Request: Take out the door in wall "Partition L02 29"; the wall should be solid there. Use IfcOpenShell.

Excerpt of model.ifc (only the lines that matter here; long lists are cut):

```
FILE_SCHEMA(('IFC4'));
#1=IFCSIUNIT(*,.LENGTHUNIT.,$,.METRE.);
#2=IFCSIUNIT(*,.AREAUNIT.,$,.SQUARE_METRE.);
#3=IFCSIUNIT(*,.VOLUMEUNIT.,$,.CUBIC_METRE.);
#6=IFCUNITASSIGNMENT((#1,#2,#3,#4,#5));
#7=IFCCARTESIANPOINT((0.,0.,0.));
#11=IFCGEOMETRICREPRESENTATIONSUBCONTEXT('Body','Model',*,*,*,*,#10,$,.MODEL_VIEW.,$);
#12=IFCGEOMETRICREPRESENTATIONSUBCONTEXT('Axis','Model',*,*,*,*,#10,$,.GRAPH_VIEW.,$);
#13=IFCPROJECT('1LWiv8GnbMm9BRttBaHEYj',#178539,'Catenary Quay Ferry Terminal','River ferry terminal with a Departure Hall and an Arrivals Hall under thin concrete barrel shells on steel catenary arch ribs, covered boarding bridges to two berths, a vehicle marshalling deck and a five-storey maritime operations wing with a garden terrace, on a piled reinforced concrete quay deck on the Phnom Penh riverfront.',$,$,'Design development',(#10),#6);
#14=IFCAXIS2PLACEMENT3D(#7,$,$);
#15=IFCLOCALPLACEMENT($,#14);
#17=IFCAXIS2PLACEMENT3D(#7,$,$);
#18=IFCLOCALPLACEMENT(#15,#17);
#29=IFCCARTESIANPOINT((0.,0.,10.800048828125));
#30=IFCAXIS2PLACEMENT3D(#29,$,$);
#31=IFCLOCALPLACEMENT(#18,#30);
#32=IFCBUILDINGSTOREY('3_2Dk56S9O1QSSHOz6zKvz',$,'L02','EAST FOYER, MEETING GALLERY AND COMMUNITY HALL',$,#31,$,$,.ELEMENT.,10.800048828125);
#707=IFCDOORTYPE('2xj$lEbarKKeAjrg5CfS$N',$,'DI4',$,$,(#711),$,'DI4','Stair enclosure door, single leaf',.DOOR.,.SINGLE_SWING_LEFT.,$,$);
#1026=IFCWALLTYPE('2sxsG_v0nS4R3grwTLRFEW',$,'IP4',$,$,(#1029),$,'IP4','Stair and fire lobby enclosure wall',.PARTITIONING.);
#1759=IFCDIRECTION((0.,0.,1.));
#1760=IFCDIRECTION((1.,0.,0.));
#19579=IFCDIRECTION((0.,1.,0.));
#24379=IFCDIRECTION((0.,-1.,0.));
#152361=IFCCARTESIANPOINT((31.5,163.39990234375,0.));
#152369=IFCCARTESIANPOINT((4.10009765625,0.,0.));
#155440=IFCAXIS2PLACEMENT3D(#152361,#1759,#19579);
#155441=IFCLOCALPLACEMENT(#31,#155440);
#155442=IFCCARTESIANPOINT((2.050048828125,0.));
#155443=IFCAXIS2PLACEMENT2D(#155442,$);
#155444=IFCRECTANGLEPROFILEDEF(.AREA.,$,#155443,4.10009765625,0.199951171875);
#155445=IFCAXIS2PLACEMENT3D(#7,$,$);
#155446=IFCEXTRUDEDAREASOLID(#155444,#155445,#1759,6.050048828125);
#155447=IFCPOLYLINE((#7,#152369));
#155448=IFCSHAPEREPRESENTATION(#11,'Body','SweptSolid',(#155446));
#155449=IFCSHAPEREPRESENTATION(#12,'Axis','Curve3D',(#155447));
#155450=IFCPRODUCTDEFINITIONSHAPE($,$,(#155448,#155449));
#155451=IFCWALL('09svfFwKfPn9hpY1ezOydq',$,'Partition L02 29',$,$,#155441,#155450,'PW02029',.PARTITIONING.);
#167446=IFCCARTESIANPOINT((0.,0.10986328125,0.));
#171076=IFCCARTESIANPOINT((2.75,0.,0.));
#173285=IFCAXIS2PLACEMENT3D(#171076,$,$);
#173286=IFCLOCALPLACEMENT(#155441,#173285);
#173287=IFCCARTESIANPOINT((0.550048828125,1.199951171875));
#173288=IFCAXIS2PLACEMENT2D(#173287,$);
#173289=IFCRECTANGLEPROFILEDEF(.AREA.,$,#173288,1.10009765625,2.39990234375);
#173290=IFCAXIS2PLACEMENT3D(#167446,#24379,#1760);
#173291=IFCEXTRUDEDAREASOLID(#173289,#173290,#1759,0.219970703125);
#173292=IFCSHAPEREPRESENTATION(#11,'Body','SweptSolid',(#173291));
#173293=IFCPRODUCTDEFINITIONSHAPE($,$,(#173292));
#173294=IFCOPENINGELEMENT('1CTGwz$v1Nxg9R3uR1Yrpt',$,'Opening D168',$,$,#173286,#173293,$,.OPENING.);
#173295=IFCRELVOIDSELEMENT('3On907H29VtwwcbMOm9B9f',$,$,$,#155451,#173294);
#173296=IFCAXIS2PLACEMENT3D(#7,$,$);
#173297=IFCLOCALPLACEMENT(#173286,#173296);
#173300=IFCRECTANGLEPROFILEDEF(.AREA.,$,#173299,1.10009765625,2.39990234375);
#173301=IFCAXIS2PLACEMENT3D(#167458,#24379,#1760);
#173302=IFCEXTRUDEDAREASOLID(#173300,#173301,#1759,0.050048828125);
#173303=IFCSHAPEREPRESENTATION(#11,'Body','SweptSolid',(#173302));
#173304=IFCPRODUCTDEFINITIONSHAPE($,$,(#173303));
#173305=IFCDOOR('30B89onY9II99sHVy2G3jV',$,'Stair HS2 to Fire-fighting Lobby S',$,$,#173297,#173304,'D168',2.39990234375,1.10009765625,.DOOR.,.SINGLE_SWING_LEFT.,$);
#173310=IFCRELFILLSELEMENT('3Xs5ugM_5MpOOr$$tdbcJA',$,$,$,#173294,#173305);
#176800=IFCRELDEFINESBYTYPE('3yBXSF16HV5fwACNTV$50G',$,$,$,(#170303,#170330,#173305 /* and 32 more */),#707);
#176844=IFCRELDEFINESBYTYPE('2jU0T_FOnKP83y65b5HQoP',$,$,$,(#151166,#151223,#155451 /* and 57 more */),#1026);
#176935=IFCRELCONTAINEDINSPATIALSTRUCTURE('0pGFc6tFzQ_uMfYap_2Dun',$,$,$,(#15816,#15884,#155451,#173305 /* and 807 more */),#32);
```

```python
import ifcopenshell
import ifcopenshell.api.feature
import ifcopenshell.api.root
import ifcopenshell.geom
import ifcopenshell.util.shape

model = ifcopenshell.open("model.ifc")
settings = ifcopenshell.geom.settings()


def volume(element):
    """Net volume in cubic metres, openings subtracted."""
    shape = ifcopenshell.geom.create_shape(settings, element)
    return ifcopenshell.util.shape.get_volume(shape.geometry)


door = model.by_guid("30B89onY9II99sHVy2G3jV")
opening = door.FillsVoids[0].RelatingOpeningElement
wall = opening.VoidsElements[0].RelatingBuildingElement
before = volume(wall)

ifcopenshell.api.root.remove_product(model, product=door)
ifcopenshell.api.feature.remove_feature(model, feature=opening)

after = volume(wall)

print(f"wall volume {before:.3f} -> {after:.3f} m3")

model.write("model_edited.ifc")
```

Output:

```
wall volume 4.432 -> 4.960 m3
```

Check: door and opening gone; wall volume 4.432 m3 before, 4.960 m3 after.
